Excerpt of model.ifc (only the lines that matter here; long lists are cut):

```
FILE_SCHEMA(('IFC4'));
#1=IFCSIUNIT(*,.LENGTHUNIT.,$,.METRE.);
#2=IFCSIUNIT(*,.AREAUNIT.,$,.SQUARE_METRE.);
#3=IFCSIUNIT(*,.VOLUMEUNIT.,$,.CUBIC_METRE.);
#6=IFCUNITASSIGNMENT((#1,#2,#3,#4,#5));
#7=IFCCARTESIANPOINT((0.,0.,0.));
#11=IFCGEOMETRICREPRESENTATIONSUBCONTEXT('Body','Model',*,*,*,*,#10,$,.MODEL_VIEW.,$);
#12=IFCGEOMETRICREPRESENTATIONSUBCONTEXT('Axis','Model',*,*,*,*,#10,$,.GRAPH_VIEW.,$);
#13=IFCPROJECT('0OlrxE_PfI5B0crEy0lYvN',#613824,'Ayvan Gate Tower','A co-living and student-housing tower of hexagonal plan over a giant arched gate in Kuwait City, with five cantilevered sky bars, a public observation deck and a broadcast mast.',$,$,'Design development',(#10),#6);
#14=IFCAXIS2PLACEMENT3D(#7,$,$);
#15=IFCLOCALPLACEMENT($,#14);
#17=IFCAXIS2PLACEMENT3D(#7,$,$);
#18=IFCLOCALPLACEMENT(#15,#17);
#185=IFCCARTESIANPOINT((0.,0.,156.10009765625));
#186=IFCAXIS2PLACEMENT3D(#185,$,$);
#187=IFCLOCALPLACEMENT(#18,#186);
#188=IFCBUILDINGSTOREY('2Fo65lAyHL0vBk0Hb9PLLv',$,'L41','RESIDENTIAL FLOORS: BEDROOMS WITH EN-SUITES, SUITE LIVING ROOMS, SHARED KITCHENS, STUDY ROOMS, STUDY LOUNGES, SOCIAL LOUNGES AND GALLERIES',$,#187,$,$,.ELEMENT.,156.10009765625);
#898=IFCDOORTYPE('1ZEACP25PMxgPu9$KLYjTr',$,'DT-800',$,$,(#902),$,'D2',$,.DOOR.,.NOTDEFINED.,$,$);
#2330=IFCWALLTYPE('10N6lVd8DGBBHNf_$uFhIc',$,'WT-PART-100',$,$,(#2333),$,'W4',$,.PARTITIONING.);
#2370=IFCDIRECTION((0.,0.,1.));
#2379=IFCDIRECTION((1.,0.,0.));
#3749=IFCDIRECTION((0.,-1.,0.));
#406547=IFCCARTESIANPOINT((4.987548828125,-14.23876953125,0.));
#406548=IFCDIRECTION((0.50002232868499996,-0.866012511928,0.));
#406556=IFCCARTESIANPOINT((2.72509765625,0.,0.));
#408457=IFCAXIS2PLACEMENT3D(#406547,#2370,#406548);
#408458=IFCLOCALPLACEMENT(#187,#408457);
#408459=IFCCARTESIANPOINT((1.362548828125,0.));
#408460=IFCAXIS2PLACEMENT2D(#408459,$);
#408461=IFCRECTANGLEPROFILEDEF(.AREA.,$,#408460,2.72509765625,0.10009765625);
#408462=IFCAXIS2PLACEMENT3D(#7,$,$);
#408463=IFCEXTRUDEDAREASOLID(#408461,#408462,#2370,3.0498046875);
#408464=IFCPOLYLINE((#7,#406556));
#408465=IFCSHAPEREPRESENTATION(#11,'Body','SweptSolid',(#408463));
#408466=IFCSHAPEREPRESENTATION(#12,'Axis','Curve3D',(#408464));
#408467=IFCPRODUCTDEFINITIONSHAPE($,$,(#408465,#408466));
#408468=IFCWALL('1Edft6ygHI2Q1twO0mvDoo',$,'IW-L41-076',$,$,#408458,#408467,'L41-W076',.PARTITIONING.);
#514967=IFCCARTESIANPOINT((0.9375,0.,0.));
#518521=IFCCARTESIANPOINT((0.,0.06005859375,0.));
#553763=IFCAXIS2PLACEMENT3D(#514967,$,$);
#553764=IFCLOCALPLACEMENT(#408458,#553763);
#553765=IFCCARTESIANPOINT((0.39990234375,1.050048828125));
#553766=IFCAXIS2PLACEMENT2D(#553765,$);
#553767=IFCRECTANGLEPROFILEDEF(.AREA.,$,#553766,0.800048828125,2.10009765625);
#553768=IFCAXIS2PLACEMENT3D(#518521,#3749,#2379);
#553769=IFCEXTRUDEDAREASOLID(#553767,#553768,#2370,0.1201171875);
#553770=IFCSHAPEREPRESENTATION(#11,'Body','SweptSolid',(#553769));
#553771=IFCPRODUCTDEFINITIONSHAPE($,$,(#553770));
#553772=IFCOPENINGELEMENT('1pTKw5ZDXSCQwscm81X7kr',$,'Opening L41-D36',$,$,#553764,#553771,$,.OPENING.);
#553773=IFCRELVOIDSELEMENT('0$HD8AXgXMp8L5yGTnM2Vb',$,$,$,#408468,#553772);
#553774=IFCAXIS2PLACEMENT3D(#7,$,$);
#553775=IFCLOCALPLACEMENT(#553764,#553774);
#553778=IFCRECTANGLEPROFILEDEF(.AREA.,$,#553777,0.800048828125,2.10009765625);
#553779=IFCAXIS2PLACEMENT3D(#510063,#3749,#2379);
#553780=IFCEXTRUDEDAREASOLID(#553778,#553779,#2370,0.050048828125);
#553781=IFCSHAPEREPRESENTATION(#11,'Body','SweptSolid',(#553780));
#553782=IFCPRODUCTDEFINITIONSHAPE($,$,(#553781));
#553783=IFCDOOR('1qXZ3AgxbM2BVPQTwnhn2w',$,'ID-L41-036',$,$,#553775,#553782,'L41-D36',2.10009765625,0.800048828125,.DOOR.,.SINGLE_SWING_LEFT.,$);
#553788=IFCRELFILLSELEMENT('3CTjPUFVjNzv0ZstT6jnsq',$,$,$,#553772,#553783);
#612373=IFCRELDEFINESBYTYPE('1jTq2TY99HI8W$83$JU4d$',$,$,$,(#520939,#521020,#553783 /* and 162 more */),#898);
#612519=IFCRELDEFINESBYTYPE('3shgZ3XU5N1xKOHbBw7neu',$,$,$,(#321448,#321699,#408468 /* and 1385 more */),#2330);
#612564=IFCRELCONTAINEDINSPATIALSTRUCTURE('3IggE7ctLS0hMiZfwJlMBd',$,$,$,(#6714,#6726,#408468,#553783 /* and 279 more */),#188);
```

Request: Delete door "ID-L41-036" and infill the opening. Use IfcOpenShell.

```python
import ifcopenshell
import ifcopenshell.api.feature
import ifcopenshell.api.root
import ifcopenshell.geom
import ifcopenshell.util.shape

model = ifcopenshell.open("model.ifc")
settings = ifcopenshell.geom.settings()


def volume(element):
    """Net volume in cubic metres, openings subtracted."""
    shape = ifcopenshell.geom.create_shape(settings, element)
    return ifcopenshell.util.shape.get_volume(shape.geometry)


door = model.by_guid("1qXZ3AgxbM2BVPQTwnhn2w")
opening = door.FillsVoids[0].RelatingOpeningElement
wall = opening.VoidsElements[0].RelatingBuildingElement
before = volume(wall)

ifcopenshell.api.root.remove_product(model, product=door)
ifcopenshell.api.feature.remove_feature(model, feature=opening)

after = volume(wall)

print(f"wall volume {before:.3f} -> {after:.3f} m3")

model.write("model_edited.ifc")
```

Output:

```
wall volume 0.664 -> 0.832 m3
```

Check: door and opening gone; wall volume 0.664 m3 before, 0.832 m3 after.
